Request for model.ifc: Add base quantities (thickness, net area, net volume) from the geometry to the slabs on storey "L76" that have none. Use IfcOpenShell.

First a look at what the model holds.

```python
import ifcopenshell
import ifcopenshell.util.element
import ifcopenshell.util.unit

model = ifcopenshell.open("model.ifc")
print(model.schema)
for unit_type in ("LENGTHUNIT", "AREAUNIT", "VOLUMEUNIT"):
    print(unit_type, ifcopenshell.util.unit.calculate_unit_scale(model, unit_type))
storey = next(s for s in model.by_type("IfcBuildingStorey") if s.Name == "L76")
slabs = [e for e in ifcopenshell.util.element.get_decomposition(storey) if e.is_a("IfcSlab")]
for e in sorted(slabs, key=lambda e: e.id()):
    print(e.id(), e.is_a(), e.Name, list(ifcopenshell.util.element.get_psets(e, qtos_only=True)), sep=" | ")
```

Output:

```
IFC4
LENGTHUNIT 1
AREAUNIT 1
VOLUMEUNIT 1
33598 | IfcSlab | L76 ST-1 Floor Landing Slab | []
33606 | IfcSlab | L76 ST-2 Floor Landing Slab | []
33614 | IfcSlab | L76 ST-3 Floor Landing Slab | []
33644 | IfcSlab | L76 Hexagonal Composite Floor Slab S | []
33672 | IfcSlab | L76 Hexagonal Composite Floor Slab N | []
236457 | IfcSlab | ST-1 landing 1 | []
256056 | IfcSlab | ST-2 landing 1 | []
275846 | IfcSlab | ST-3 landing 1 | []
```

```python
import ifcopenshell
import ifcopenshell.api.pset
import ifcopenshell.geom
import ifcopenshell.util.element
import ifcopenshell.util.shape
import ifcopenshell.util.unit

model = ifcopenshell.open("model.ifc")
unit_scale = ifcopenshell.util.unit.calculate_unit_scale(model)
area_scale = ifcopenshell.util.unit.calculate_unit_scale(model, "AREAUNIT")
volume_scale = ifcopenshell.util.unit.calculate_unit_scale(model, "VOLUMEUNIT")
settings = ifcopenshell.geom.settings()

storey = next(s for s in model.by_type("IfcBuildingStorey") if s.Name == "L76")
slabs = [e for e in ifcopenshell.util.element.get_decomposition(storey) if e.is_a("IfcSlab")]

for e in sorted(slabs, key=lambda e: e.id()):
    if ifcopenshell.util.element.get_psets(e, qtos_only=True, should_inherit=False):
        continue
    # Geometry comes back in metres, in the element's own axes.
    shape = ifcopenshell.geom.create_shape(settings, e)
    values = {
        "Width": ifcopenshell.util.shape.get_z(shape.geometry) / unit_scale,
        "NetArea": ifcopenshell.util.shape.get_footprint_area(shape.geometry) / area_scale,
        "NetVolume": ifcopenshell.util.shape.get_volume(shape.geometry) / volume_scale,
    }
    qto = ifcopenshell.api.pset.add_qto(model, product=e, name="Qto_SlabBaseQuantities")
    ifcopenshell.api.pset.edit_qto(model, qto=qto, properties=values)
    print(e.id(), {k: round(v, 3) for k, v in values.items()})

model.write("model-out.ifc")
```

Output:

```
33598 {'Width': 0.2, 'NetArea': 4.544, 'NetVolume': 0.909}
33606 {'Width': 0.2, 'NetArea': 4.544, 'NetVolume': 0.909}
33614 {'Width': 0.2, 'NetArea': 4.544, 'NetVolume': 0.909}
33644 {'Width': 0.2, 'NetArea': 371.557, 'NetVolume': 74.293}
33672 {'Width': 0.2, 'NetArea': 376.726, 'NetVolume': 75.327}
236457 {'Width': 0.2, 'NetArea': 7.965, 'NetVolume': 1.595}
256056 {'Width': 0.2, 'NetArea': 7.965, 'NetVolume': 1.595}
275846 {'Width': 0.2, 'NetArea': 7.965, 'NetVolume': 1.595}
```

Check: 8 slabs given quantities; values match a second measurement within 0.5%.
